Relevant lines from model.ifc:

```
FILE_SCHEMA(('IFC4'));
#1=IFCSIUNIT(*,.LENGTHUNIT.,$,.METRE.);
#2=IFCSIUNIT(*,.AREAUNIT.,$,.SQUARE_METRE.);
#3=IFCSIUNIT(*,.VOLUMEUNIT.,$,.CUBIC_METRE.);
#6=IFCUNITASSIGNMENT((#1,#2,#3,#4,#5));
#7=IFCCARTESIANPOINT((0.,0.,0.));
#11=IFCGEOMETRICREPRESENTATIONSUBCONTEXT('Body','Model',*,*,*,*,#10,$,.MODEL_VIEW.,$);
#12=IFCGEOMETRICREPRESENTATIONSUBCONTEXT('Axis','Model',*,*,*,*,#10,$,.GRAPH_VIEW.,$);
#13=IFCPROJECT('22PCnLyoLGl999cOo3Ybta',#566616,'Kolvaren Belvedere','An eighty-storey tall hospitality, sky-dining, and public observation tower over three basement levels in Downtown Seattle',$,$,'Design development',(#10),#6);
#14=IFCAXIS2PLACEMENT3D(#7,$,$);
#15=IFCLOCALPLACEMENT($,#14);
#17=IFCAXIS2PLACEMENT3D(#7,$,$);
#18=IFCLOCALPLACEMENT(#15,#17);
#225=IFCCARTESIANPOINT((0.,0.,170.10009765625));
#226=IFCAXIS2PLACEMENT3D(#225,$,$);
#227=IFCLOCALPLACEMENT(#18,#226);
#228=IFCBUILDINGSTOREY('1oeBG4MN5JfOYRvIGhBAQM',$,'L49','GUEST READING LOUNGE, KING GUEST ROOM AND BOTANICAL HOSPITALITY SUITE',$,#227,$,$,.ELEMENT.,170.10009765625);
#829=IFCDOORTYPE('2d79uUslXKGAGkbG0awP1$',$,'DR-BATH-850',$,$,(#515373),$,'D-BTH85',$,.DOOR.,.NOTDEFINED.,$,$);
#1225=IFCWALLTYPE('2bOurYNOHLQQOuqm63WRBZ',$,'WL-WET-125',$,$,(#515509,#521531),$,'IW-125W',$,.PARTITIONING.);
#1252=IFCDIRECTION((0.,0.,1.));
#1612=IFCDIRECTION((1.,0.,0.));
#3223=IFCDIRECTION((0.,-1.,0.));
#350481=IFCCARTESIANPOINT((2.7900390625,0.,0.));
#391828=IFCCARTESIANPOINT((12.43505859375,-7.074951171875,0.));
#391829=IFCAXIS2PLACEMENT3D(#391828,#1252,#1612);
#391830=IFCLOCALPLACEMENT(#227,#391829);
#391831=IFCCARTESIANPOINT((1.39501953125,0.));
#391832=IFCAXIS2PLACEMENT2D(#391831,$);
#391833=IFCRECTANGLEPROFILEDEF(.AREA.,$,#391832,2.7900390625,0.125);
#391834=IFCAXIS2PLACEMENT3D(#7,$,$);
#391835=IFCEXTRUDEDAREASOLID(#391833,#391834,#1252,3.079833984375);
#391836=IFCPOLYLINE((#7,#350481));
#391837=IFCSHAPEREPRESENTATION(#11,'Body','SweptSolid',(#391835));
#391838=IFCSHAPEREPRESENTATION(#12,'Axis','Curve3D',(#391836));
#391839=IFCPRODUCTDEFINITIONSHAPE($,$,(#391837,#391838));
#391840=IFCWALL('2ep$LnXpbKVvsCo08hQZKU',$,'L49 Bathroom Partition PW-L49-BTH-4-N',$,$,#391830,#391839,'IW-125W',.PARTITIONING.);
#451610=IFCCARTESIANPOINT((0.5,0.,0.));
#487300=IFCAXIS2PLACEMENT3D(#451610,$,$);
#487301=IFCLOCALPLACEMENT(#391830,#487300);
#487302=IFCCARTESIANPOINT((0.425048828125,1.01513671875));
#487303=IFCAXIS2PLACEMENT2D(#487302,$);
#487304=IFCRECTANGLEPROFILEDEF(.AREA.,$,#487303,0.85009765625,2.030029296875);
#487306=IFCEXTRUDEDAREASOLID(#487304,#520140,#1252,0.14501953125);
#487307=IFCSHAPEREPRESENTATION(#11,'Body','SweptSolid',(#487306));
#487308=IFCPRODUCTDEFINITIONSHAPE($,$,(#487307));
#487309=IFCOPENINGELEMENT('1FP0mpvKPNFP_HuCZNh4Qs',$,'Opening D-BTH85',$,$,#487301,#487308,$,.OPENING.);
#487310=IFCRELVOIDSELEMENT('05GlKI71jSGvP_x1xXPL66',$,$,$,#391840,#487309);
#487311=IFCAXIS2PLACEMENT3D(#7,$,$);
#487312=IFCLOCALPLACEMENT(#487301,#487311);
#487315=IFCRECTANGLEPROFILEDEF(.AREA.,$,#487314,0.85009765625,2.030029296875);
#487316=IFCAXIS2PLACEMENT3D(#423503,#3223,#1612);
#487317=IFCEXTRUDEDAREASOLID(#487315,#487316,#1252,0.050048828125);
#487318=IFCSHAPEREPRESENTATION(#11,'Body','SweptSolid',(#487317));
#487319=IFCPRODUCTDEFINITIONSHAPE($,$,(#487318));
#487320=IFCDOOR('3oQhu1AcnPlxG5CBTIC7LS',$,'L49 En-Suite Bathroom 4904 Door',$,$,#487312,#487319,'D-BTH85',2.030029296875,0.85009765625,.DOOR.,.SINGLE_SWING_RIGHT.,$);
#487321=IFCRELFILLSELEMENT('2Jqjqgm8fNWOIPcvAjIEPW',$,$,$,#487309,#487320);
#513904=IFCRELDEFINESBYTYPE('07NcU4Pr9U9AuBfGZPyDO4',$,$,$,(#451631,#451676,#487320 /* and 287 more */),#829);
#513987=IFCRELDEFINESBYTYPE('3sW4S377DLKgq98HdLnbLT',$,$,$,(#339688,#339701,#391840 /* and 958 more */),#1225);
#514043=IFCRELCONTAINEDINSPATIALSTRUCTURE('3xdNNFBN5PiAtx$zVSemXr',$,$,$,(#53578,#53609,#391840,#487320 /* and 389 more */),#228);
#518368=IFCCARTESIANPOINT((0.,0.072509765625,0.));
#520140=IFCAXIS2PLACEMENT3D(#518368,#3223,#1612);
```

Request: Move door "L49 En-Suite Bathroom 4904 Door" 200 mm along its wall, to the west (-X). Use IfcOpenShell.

```python
import ifcopenshell
import ifcopenshell.api.geometry
import ifcopenshell.util.placement
import ifcopenshell.util.unit

model = ifcopenshell.open("model.ifc")
unit_scale = ifcopenshell.util.unit.calculate_unit_scale(model)

door = model.by_id(487320)
opening = door.FillsVoids[0].RelatingOpeningElement
wall = opening.VoidsElements[0].RelatingBuildingElement

wall_matrix = ifcopenshell.util.placement.get_local_placement(wall.ObjectPlacement)
shift = wall_matrix[:3, 0] * -0.2 / unit_scale
before = ifcopenshell.util.placement.get_local_placement(door.ObjectPlacement)[:3, 3].copy()

# The door is placed relative to its opening, so it follows when the opening moves.
matrix = ifcopenshell.util.placement.get_local_placement(opening.ObjectPlacement)
matrix[:3, 3] += shift
ifcopenshell.api.geometry.edit_object_placement(
    model, product=opening, matrix=matrix, is_si=False, should_transform_children=True
)

after = ifcopenshell.util.placement.get_local_placement(door.ObjectPlacement)[:3, 3]
print("door moved by", (after - before).round(3) + 0.0)

model.write("model-out.ifc")
```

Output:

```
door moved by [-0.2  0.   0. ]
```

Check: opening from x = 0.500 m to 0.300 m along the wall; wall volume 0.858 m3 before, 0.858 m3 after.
